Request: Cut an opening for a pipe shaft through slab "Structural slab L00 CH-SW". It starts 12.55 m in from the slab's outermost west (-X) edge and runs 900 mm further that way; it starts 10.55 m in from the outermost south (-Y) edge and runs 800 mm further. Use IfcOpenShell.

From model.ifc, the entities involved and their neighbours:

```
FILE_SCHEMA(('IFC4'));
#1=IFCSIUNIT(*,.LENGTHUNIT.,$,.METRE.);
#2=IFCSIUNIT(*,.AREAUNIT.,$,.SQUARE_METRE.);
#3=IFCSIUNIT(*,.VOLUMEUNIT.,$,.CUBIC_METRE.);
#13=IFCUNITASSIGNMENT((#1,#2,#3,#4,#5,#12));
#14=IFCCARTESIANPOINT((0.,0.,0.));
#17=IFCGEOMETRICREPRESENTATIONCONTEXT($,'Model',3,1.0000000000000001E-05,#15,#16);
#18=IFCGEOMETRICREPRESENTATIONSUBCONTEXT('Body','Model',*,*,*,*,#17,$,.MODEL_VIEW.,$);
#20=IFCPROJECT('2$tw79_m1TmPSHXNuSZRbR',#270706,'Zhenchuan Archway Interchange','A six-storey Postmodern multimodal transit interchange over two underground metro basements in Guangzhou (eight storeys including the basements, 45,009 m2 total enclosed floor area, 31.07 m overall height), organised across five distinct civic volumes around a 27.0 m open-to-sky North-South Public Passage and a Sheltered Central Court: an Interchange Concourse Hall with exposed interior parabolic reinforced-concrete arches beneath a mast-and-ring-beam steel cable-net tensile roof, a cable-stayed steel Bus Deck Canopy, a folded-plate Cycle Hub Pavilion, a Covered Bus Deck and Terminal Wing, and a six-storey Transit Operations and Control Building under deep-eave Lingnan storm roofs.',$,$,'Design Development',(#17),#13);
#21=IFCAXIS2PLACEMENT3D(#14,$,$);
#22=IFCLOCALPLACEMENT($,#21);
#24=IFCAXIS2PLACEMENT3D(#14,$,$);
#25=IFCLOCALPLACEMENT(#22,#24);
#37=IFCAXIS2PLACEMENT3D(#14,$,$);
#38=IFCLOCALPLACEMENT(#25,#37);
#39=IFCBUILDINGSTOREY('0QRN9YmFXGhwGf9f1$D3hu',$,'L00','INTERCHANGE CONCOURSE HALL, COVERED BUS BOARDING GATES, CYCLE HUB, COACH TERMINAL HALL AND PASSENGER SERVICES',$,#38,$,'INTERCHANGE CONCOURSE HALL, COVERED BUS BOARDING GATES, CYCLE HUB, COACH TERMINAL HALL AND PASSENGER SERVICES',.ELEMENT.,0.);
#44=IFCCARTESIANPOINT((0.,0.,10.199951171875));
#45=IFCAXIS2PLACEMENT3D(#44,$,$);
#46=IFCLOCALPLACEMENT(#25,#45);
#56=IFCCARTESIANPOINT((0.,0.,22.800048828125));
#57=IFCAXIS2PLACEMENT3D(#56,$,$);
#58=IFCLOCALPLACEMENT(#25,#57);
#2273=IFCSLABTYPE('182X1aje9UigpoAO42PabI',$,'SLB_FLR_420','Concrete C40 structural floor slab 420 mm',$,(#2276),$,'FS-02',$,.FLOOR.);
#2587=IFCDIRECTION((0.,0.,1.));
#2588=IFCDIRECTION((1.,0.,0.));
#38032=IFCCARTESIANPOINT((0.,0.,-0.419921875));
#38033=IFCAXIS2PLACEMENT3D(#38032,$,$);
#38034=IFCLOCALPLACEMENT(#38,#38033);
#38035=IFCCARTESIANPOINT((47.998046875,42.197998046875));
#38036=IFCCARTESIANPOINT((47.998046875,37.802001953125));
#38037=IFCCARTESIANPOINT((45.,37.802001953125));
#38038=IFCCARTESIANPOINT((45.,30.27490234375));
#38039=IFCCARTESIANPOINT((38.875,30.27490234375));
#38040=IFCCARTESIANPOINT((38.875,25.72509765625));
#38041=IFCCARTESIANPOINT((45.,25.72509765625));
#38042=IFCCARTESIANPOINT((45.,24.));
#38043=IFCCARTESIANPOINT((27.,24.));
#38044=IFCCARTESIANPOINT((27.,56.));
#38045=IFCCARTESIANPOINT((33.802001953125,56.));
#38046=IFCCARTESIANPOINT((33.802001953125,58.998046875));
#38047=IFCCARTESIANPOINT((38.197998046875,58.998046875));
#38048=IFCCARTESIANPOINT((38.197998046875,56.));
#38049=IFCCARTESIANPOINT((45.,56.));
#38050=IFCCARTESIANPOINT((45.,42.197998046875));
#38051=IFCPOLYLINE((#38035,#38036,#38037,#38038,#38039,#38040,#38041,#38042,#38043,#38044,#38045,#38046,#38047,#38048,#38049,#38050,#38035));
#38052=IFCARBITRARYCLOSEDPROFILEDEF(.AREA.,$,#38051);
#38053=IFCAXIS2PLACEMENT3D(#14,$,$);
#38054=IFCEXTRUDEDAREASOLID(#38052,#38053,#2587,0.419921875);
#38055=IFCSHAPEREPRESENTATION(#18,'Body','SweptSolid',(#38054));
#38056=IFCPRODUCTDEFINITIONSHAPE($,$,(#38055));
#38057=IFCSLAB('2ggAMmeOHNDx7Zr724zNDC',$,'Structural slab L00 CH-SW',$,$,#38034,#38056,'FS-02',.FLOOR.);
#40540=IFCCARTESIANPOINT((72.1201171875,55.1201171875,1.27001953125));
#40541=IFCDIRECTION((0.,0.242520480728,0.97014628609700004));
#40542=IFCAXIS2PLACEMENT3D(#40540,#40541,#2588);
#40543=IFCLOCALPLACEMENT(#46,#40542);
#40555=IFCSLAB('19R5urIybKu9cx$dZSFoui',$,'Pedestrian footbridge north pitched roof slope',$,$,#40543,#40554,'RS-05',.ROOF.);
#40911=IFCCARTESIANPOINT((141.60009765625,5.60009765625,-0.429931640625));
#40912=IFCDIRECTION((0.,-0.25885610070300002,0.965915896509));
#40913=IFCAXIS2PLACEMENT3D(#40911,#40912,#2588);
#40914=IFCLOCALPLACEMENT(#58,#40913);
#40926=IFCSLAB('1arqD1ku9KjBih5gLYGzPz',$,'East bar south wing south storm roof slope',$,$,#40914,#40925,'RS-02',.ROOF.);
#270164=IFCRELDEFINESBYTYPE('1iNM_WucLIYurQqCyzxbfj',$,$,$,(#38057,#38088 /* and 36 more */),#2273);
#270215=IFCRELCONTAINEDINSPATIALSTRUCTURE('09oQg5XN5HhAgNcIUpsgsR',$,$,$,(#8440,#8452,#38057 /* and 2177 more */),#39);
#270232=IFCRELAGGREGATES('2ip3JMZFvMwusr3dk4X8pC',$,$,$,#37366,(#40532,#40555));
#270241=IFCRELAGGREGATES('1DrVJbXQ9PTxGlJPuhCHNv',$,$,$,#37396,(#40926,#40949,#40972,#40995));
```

```python
import numpy as np
import ifcopenshell
import ifcopenshell.api.feature
import ifcopenshell.api.geometry
import ifcopenshell.api.root
import ifcopenshell.geom
import ifcopenshell.util.placement
import ifcopenshell.util.representation
import ifcopenshell.util.shape
import ifcopenshell.util.unit

model = ifcopenshell.open("model.ifc")
unit_scale = ifcopenshell.util.unit.calculate_unit_scale(model)
settings = ifcopenshell.geom.settings()


def volume(element):
    """Net volume in cubic metres, openings subtracted."""
    shape = ifcopenshell.geom.create_shape(settings, element)
    return ifcopenshell.util.shape.get_volume(shape.geometry)


slab = model.by_guid("2ggAMmeOHNDx7Zr724zNDC")
before = volume(slab)

# Extent in the slab's own axes, in metres. The edges named are its -X and -Y sides.
slab_shape = ifcopenshell.geom.create_shape(settings, slab)
vertices = ifcopenshell.util.shape.get_vertices(slab_shape.geometry)
x_min, y_min, bottom = vertices.min(axis=0)
top = vertices[:, 2].max()

opening = ifcopenshell.api.root.create_entity(model, ifc_class="IfcOpeningElement", name="Pipe shaft opening", predefined_type="OPENING")
context = ifcopenshell.util.representation.get_context(model, "Model", "Body", "MODEL_VIEW")
width, depth = 0.9, 0.8
outline = [(0.0, 0.0), (width, 0.0), (width, depth), (0.0, depth), (0.0, 0.0)]
# Overshoot both faces by 50 mm so the cut is clean.
shape = ifcopenshell.api.geometry.add_slab_representation(
    model, context=context, depth=top - bottom + 0.1, polyline=outline
)
ifcopenshell.api.geometry.assign_representation(model, product=opening, representation=shape)

matrix = ifcopenshell.util.placement.get_local_placement(slab.ObjectPlacement)
matrix[:, 3] = matrix @ np.append(np.array([x_min + 12.55, y_min + 10.55, bottom - 0.05]) / unit_scale, 1.0)
ifcopenshell.api.geometry.edit_object_placement(model, product=opening, matrix=matrix, is_si=False)
ifcopenshell.api.feature.add_feature(model, feature=opening, element=slab)

after = volume(slab)

print(f"slab volume {before:.3f} -> {after:.3f} m3")

model.write("model_v2.ifc")
```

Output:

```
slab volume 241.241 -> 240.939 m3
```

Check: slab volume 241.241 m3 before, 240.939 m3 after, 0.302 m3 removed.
